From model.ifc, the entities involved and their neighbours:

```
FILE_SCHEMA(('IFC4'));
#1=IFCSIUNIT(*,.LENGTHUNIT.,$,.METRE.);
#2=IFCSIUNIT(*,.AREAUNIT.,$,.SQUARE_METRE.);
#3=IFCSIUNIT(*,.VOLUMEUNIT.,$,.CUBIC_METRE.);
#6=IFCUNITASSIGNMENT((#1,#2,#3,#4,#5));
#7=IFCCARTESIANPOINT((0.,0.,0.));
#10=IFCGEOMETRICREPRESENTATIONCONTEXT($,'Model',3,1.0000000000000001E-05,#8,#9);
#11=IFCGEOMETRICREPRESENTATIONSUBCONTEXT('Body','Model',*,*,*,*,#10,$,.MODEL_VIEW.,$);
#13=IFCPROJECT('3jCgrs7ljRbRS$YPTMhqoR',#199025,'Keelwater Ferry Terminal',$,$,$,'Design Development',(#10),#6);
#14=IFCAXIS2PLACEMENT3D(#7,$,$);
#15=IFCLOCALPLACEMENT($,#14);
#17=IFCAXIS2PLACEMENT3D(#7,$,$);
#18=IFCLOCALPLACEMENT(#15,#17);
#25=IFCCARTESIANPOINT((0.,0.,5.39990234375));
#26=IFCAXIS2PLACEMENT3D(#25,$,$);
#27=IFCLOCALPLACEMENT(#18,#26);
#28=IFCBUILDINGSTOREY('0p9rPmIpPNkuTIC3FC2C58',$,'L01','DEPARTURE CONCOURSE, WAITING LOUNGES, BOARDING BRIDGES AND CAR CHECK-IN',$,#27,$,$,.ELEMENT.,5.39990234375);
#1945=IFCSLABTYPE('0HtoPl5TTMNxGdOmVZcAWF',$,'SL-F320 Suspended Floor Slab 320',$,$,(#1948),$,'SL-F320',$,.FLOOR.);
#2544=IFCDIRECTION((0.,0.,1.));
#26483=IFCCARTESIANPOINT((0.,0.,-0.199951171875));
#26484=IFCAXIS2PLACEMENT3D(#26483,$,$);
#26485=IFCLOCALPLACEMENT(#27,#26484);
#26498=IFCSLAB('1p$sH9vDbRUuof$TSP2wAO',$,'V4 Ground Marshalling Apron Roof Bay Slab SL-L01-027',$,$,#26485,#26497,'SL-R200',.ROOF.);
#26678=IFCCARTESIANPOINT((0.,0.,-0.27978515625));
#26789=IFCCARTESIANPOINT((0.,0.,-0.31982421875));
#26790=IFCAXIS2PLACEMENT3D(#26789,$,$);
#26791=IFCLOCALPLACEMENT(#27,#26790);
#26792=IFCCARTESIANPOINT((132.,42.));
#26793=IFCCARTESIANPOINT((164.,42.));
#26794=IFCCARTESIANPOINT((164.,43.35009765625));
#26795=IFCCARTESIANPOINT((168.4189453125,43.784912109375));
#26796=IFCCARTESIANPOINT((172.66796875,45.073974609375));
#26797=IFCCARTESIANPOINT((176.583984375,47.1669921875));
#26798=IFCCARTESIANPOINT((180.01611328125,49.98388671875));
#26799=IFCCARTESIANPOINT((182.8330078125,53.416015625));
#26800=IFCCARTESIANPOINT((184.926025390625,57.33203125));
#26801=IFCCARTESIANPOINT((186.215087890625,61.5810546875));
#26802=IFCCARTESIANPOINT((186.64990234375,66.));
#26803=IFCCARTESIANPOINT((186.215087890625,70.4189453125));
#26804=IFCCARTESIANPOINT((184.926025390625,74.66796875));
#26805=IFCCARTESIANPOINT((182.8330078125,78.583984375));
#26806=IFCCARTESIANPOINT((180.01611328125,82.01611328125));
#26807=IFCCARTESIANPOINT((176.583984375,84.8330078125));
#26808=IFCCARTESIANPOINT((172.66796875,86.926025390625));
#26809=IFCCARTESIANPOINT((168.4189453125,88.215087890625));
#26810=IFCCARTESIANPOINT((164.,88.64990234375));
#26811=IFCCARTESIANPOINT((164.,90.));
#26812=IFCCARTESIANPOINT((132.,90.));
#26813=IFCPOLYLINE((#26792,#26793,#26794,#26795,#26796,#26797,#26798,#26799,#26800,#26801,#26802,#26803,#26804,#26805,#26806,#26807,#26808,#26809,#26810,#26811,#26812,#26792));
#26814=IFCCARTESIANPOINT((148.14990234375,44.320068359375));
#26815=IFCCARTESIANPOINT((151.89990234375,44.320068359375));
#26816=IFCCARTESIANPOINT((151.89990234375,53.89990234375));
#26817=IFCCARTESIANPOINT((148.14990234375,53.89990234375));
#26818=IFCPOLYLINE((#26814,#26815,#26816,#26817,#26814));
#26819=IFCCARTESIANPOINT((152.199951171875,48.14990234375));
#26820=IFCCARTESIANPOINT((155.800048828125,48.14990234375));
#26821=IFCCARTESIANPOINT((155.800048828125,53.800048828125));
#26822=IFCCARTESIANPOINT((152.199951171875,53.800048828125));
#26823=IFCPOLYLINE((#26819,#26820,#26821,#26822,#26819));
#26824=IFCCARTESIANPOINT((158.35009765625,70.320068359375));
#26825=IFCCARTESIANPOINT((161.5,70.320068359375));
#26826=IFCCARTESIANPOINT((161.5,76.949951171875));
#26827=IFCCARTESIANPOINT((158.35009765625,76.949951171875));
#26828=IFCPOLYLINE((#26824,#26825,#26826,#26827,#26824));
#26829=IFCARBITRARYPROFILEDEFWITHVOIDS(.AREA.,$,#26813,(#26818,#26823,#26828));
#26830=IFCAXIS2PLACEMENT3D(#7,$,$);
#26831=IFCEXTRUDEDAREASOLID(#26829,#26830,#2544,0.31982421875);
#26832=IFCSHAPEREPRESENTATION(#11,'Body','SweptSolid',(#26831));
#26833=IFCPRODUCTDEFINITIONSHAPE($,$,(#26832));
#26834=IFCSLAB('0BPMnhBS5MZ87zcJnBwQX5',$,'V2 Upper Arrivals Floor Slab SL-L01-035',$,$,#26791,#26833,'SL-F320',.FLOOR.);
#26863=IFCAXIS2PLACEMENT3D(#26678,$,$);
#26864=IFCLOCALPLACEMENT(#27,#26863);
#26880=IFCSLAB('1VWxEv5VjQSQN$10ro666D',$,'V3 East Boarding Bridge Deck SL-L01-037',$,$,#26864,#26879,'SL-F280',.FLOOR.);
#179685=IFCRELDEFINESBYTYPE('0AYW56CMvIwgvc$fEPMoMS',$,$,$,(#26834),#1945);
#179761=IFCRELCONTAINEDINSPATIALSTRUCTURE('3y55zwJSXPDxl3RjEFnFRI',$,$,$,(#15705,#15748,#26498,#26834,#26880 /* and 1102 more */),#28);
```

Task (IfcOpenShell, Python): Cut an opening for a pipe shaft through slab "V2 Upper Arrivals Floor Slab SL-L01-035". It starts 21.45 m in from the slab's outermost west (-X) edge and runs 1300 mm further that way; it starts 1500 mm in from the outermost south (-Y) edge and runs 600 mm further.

```python
import numpy as np
import ifcopenshell
import ifcopenshell.api.feature
import ifcopenshell.api.geometry
import ifcopenshell.api.root
import ifcopenshell.geom
import ifcopenshell.util.placement
import ifcopenshell.util.representation
import ifcopenshell.util.shape
import ifcopenshell.util.unit

model = ifcopenshell.open("model.ifc")
unit_scale = ifcopenshell.util.unit.calculate_unit_scale(model)
settings = ifcopenshell.geom.settings()


def volume(element):
    """Net volume in cubic metres, openings subtracted."""
    shape = ifcopenshell.geom.create_shape(settings, element)
    return ifcopenshell.util.shape.get_volume(shape.geometry)


slab = model.by_id(26834)
before = volume(slab)

# Extent in the slab's own axes, in metres. The edges named are its -X and -Y sides.
slab_shape = ifcopenshell.geom.create_shape(settings, slab)
vertices = ifcopenshell.util.shape.get_vertices(slab_shape.geometry)
x_min, y_min, bottom = vertices.min(axis=0)
top = vertices[:, 2].max()

opening = ifcopenshell.api.root.create_entity(model, ifc_class="IfcOpeningElement", name="Pipe shaft opening", predefined_type="OPENING")
context = ifcopenshell.util.representation.get_context(model, "Model", "Body", "MODEL_VIEW")
width, depth = 1.3, 0.6
outline = [(0.0, 0.0), (width, 0.0), (width, depth), (0.0, depth), (0.0, 0.0)]
# Overshoot both faces by 50 mm so the cut is clean.
shape = ifcopenshell.api.geometry.add_slab_representation(
    model, context=context, depth=top - bottom + 0.1, polyline=outline
)
ifcopenshell.api.geometry.assign_representation(model, product=opening, representation=shape)

matrix = ifcopenshell.util.placement.get_local_placement(slab.ObjectPlacement)
matrix[:, 3] = matrix @ np.append(np.array([x_min + 21.45, y_min + 1.5, bottom - 0.05]) / unit_scale, 1.0)
ifcopenshell.api.geometry.edit_object_placement(model, product=opening, matrix=matrix, is_si=False)
ifcopenshell.api.feature.add_feature(model, feature=opening, element=slab)

after = volume(slab)

print(f"slab volume {before:.3f} -> {after:.3f} m3")

model.write("model_rev.ifc")
```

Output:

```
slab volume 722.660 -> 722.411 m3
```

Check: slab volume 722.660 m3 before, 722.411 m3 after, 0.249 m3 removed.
